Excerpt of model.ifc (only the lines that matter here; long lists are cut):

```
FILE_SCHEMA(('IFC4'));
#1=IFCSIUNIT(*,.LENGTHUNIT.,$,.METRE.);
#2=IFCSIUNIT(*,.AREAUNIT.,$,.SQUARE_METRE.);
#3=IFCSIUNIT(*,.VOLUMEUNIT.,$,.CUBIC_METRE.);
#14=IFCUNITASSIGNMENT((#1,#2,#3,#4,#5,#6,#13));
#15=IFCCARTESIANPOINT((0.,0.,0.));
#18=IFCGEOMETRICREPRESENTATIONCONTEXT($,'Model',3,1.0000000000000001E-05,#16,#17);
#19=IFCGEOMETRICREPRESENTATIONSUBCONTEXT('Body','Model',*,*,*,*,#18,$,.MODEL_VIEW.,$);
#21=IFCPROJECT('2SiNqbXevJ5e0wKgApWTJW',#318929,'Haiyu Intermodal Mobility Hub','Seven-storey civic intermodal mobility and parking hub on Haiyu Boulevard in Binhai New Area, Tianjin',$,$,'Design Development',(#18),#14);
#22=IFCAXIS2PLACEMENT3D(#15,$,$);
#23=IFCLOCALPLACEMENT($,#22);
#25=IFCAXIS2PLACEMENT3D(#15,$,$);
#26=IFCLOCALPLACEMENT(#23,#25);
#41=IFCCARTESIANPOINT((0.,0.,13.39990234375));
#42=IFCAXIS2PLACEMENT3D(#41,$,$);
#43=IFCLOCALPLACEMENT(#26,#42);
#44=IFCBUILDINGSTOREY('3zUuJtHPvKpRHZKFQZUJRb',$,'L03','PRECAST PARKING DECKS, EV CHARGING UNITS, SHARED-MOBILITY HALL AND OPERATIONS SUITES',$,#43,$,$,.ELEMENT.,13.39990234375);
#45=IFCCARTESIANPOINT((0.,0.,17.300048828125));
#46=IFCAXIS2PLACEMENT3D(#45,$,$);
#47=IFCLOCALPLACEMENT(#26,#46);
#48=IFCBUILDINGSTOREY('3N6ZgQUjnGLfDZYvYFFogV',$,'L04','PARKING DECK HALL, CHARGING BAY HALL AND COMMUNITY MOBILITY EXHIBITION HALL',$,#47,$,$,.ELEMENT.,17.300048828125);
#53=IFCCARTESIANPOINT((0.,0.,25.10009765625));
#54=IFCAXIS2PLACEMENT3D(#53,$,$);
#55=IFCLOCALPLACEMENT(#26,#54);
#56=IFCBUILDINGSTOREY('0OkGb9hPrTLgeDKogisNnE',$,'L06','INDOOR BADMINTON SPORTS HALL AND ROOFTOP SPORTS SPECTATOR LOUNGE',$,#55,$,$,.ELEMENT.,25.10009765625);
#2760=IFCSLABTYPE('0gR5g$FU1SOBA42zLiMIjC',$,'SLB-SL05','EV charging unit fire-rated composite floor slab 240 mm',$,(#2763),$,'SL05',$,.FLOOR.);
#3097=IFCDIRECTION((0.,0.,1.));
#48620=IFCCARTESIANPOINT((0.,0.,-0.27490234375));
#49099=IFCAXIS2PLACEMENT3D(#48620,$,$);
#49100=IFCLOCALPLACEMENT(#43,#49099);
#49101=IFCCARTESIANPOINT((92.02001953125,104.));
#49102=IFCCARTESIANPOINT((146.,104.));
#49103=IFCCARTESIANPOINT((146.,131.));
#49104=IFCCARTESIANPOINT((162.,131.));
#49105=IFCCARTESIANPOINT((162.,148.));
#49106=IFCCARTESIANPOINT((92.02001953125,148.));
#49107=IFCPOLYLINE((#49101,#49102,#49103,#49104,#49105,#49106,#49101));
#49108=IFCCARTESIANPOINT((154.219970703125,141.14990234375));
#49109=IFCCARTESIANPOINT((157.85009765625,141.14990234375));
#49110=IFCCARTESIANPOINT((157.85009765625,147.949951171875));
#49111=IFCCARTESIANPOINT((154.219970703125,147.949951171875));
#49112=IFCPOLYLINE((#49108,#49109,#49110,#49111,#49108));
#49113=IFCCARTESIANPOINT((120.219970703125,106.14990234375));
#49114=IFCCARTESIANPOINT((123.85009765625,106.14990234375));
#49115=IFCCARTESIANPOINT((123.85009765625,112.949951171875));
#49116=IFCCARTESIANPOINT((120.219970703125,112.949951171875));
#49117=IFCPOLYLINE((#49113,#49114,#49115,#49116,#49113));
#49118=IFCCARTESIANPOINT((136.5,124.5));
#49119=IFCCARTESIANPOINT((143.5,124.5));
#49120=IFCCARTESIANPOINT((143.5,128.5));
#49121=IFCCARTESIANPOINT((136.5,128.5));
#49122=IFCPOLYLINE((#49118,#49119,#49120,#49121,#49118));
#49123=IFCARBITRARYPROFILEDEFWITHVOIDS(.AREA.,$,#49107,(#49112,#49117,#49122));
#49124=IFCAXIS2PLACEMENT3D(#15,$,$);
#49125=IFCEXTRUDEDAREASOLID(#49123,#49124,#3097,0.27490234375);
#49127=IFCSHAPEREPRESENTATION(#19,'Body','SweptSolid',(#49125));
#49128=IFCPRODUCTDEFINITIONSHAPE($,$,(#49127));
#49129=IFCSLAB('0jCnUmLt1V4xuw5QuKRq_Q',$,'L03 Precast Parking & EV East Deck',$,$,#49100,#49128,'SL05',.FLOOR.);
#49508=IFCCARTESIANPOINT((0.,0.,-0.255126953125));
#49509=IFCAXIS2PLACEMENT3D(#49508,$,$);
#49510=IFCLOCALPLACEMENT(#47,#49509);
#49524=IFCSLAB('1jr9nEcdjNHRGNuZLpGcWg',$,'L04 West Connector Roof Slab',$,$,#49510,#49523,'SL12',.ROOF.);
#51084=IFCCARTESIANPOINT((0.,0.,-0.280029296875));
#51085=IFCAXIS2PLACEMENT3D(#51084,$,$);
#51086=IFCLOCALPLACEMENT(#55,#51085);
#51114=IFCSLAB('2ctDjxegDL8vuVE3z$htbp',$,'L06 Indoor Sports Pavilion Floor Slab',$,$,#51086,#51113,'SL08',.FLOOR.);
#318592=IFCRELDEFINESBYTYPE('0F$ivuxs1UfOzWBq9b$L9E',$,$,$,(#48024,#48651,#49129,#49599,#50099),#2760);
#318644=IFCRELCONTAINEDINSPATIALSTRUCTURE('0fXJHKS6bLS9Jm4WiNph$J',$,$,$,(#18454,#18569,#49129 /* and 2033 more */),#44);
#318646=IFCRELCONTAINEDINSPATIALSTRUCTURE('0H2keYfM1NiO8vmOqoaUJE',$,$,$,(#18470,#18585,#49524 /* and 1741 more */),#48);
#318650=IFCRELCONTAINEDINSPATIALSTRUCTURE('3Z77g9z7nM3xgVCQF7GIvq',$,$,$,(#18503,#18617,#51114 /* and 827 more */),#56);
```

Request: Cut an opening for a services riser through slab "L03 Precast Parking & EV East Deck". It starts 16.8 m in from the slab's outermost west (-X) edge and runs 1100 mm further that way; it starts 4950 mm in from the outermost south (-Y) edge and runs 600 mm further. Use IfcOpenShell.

```python
import numpy as np
import ifcopenshell
import ifcopenshell.api.feature
import ifcopenshell.api.geometry
import ifcopenshell.api.root
import ifcopenshell.geom
import ifcopenshell.util.placement
import ifcopenshell.util.representation
import ifcopenshell.util.shape
import ifcopenshell.util.unit

model = ifcopenshell.open("model.ifc")
unit_scale = ifcopenshell.util.unit.calculate_unit_scale(model)
settings = ifcopenshell.geom.settings()


def volume(element):
    """Net volume in cubic metres, openings subtracted."""
    shape = ifcopenshell.geom.create_shape(settings, element)
    return ifcopenshell.util.shape.get_volume(shape.geometry)


slab = model.by_guid("0jCnUmLt1V4xuw5QuKRq_Q")
before = volume(slab)

# Extent in the slab's own axes, in metres. The edges named are its -X and -Y sides.
slab_shape = ifcopenshell.geom.create_shape(settings, slab)
vertices = ifcopenshell.util.shape.get_vertices(slab_shape.geometry)
x_min, y_min, bottom = vertices.min(axis=0)
top = vertices[:, 2].max()

opening = ifcopenshell.api.root.create_entity(model, ifc_class="IfcOpeningElement", name="Services riser opening", predefined_type="OPENING")
context = ifcopenshell.util.representation.get_context(model, "Model", "Body", "MODEL_VIEW")
width, depth = 1.1, 0.6
outline = [(0.0, 0.0), (width, 0.0), (width, depth), (0.0, depth), (0.0, 0.0)]
# Overshoot both faces by 50 mm so the cut is clean.
shape = ifcopenshell.api.geometry.add_slab_representation(
    model, context=context, depth=top - bottom + 0.1, polyline=outline
)
ifcopenshell.api.geometry.assign_representation(model, product=opening, representation=shape)

matrix = ifcopenshell.util.placement.get_local_placement(slab.ObjectPlacement)
matrix[:, 3] = matrix @ np.append(np.array([x_min + 16.8, y_min + 4.95, bottom - 0.05]) / unit_scale, 1.0)
ifcopenshell.api.geometry.edit_object_placement(model, product=opening, matrix=matrix, is_si=False)
ifcopenshell.api.feature.add_feature(model, feature=opening, element=slab)

after = volume(slab)

print(f"slab volume {before:.3f} -> {after:.3f} m3")

model.write("model_rev.ifc")
```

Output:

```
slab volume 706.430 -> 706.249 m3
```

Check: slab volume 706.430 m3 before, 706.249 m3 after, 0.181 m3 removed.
